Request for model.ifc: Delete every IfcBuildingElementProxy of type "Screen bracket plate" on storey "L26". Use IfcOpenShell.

First a look at what the model holds.

```python
import ifcopenshell
import ifcopenshell.util.element

model = ifcopenshell.open("model.ifc")
print(model.schema)
storey = next(s for s in model.by_type("IfcBuildingStorey") if s.Name == "L26")
proxies = [e for e in ifcopenshell.util.element.get_decomposition(storey) if e.is_a("IfcBuildingElementProxy")]
seen = {}
for e in proxies:
    element_type = ifcopenshell.util.element.get_type(e)
    name = element_type.Name if element_type not in (None, e) else None
    seen[name] = seen.get(name, 0) + 1
for name, count in sorted(seen.items(), key=str):
    print(count, "x", name)
```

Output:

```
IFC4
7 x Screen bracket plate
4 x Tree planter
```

```python
import ifcopenshell
import ifcopenshell.api.root
import ifcopenshell.util.element

model = ifcopenshell.open("model.ifc")

storey = next(s for s in model.by_type("IfcBuildingStorey") if s.Name == "L26")
proxies = [e for e in ifcopenshell.util.element.get_decomposition(storey) if e.is_a("IfcBuildingElementProxy")]
targets = [e for e in proxies if (t := ifcopenshell.util.element.get_type(e)) not in (None, e) and t.Name == "Screen bracket plate"]

for e in targets:
    ifcopenshell.api.root.remove_product(model, product=e)
print(len(targets), "removed")

model.write("model_edited.ifc")
```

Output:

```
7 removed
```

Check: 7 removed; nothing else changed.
